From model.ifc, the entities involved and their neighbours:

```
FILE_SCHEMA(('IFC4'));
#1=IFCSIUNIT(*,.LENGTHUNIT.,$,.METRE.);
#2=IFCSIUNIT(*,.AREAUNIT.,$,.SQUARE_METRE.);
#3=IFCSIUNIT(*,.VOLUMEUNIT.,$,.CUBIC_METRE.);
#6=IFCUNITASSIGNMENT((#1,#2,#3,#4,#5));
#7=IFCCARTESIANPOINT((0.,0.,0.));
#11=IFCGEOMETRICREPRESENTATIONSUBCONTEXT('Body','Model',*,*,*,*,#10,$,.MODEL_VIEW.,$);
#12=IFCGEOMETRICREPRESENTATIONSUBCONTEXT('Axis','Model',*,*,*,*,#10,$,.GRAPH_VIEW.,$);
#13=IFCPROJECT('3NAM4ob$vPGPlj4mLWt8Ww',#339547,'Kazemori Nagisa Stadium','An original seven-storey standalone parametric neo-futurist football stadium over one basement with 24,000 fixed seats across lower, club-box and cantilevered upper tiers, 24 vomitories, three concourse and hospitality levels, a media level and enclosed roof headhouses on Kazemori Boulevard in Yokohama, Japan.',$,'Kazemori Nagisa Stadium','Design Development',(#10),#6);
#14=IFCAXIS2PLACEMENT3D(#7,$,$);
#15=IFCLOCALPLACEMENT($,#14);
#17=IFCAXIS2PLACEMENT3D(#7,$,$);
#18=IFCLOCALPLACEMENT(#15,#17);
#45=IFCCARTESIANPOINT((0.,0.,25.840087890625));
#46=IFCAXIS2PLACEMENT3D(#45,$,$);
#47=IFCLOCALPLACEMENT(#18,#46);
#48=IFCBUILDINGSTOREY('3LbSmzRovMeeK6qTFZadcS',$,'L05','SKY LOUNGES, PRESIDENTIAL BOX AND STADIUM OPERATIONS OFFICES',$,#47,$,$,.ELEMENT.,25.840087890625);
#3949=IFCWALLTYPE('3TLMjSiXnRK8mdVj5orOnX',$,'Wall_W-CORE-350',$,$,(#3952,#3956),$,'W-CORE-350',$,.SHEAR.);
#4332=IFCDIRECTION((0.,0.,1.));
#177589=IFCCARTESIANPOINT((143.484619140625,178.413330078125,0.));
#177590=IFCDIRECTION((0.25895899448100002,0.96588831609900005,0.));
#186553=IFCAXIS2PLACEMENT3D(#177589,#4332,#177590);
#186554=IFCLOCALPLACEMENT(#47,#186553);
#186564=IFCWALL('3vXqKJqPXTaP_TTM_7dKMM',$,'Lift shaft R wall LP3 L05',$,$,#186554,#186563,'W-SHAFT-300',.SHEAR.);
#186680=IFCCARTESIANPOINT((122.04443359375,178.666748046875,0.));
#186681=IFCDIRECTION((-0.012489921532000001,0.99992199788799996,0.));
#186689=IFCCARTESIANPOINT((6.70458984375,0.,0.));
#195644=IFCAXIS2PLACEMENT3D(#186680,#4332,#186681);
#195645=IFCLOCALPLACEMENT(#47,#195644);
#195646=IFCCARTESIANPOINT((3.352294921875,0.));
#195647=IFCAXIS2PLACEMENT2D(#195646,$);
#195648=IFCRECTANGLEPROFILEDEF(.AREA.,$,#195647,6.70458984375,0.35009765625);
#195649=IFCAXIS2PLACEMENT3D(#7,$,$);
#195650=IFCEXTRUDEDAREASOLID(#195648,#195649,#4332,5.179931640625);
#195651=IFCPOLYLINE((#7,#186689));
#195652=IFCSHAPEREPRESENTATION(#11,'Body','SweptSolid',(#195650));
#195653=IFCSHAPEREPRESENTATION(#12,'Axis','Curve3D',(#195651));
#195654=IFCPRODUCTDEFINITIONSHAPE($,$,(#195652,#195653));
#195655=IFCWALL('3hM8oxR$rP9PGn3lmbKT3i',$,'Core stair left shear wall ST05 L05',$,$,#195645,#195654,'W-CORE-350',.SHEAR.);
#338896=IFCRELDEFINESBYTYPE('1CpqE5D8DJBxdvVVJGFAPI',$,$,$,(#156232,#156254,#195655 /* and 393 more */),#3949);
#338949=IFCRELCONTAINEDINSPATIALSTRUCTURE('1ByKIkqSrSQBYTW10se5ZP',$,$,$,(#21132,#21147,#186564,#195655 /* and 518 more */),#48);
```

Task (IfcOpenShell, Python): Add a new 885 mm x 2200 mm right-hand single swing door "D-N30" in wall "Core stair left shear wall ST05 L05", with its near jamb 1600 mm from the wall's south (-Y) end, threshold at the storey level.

```python
import numpy as np
import ifcopenshell
import ifcopenshell.api.feature
import ifcopenshell.api.geometry
import ifcopenshell.api.root
import ifcopenshell.api.spatial
import ifcopenshell.geom
import ifcopenshell.util.element
import ifcopenshell.util.placement
import ifcopenshell.util.representation
import ifcopenshell.util.shape
import ifcopenshell.util.unit

model = ifcopenshell.open("model.ifc")
unit_scale = ifcopenshell.util.unit.calculate_unit_scale(model)
settings = ifcopenshell.geom.settings()


def volume(element):
    """Net volume in cubic metres, openings subtracted."""
    shape = ifcopenshell.geom.create_shape(settings, element)
    return ifcopenshell.util.shape.get_volume(shape.geometry)


wall = model.by_guid("3hM8oxR$rP9PGn3lmbKT3i")
storey = ifcopenshell.util.element.get_container(wall, ifc_class="IfcBuildingStorey")
context = ifcopenshell.util.representation.get_context(model, "Model", "Body", "MODEL_VIEW")
before = volume(wall)

width, height, from_end, sill = 0.885, 2.2, 1.6, 0.0  # metres

# The wall runs along its own X axis, and the end named is its -X end.
wall_shape = ifcopenshell.geom.create_shape(settings, wall)
x, y, z = ifcopenshell.util.shape.get_vertices(wall_shape.geometry).T
start = x.min() + from_end
face, thickness = float(y.min()), float(y.max() - y.min())
wall_matrix = ifcopenshell.util.placement.get_local_placement(wall.ObjectPlacement)
level = ifcopenshell.util.placement.get_local_placement(storey.ObjectPlacement)[2, 3]


def in_wall(x, y):
    """Placement at x, y metres in the wall's axes, at sill height."""
    matrix = wall_matrix.copy()
    matrix[:, 3] = wall_matrix @ np.array([x / unit_scale, y / unit_scale, 0.0, 1.0])
    matrix[2, 3] = level + sill / unit_scale
    return matrix


# Opening: a box that overshoots both wall faces by 50 mm.
opening = ifcopenshell.api.root.create_entity(model, ifc_class="IfcOpeningElement", predefined_type="OPENING")
box = ifcopenshell.api.geometry.add_wall_representation(
    model, context=context, length=width, height=height, thickness=thickness + 0.1
)
ifcopenshell.api.geometry.assign_representation(model, product=opening, representation=box)
ifcopenshell.api.geometry.edit_object_placement(model, product=opening, matrix=in_wall(start, face - 0.05), is_si=False)
ifcopenshell.api.feature.add_feature(model, feature=opening, element=wall)

door = ifcopenshell.api.root.create_entity(model, ifc_class="IfcDoor", name="D-N30", predefined_type="DOOR")
door.OverallWidth, door.OverallHeight = width / unit_scale, height / unit_scale
door.OperationType = "SINGLE_SWING_RIGHT"
body = ifcopenshell.api.geometry.add_door_representation(
    model,
    context=context,
    overall_width=door.OverallWidth,
    overall_height=door.OverallHeight,
    operation_type="SINGLE_SWING_RIGHT",
    lining_properties={"LiningDepth": thickness / unit_scale, "ThresholdDepth": thickness / unit_scale},
)
ifcopenshell.api.geometry.assign_representation(model, product=door, representation=body)
ifcopenshell.api.spatial.assign_container(model, products=[door], relating_structure=storey)
ifcopenshell.api.feature.add_filling(model, opening=opening, element=door)

# The lining spans the wall, so the door starts at the wall face.
ifcopenshell.api.geometry.edit_object_placement(model, product=door, matrix=in_wall(start, face), is_si=False)

after = volume(wall)

print(f"wall volume {before:.3f} -> {after:.3f} m3")

model.write("model_updated.ifc")
```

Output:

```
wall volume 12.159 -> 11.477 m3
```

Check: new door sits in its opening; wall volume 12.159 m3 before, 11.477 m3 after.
